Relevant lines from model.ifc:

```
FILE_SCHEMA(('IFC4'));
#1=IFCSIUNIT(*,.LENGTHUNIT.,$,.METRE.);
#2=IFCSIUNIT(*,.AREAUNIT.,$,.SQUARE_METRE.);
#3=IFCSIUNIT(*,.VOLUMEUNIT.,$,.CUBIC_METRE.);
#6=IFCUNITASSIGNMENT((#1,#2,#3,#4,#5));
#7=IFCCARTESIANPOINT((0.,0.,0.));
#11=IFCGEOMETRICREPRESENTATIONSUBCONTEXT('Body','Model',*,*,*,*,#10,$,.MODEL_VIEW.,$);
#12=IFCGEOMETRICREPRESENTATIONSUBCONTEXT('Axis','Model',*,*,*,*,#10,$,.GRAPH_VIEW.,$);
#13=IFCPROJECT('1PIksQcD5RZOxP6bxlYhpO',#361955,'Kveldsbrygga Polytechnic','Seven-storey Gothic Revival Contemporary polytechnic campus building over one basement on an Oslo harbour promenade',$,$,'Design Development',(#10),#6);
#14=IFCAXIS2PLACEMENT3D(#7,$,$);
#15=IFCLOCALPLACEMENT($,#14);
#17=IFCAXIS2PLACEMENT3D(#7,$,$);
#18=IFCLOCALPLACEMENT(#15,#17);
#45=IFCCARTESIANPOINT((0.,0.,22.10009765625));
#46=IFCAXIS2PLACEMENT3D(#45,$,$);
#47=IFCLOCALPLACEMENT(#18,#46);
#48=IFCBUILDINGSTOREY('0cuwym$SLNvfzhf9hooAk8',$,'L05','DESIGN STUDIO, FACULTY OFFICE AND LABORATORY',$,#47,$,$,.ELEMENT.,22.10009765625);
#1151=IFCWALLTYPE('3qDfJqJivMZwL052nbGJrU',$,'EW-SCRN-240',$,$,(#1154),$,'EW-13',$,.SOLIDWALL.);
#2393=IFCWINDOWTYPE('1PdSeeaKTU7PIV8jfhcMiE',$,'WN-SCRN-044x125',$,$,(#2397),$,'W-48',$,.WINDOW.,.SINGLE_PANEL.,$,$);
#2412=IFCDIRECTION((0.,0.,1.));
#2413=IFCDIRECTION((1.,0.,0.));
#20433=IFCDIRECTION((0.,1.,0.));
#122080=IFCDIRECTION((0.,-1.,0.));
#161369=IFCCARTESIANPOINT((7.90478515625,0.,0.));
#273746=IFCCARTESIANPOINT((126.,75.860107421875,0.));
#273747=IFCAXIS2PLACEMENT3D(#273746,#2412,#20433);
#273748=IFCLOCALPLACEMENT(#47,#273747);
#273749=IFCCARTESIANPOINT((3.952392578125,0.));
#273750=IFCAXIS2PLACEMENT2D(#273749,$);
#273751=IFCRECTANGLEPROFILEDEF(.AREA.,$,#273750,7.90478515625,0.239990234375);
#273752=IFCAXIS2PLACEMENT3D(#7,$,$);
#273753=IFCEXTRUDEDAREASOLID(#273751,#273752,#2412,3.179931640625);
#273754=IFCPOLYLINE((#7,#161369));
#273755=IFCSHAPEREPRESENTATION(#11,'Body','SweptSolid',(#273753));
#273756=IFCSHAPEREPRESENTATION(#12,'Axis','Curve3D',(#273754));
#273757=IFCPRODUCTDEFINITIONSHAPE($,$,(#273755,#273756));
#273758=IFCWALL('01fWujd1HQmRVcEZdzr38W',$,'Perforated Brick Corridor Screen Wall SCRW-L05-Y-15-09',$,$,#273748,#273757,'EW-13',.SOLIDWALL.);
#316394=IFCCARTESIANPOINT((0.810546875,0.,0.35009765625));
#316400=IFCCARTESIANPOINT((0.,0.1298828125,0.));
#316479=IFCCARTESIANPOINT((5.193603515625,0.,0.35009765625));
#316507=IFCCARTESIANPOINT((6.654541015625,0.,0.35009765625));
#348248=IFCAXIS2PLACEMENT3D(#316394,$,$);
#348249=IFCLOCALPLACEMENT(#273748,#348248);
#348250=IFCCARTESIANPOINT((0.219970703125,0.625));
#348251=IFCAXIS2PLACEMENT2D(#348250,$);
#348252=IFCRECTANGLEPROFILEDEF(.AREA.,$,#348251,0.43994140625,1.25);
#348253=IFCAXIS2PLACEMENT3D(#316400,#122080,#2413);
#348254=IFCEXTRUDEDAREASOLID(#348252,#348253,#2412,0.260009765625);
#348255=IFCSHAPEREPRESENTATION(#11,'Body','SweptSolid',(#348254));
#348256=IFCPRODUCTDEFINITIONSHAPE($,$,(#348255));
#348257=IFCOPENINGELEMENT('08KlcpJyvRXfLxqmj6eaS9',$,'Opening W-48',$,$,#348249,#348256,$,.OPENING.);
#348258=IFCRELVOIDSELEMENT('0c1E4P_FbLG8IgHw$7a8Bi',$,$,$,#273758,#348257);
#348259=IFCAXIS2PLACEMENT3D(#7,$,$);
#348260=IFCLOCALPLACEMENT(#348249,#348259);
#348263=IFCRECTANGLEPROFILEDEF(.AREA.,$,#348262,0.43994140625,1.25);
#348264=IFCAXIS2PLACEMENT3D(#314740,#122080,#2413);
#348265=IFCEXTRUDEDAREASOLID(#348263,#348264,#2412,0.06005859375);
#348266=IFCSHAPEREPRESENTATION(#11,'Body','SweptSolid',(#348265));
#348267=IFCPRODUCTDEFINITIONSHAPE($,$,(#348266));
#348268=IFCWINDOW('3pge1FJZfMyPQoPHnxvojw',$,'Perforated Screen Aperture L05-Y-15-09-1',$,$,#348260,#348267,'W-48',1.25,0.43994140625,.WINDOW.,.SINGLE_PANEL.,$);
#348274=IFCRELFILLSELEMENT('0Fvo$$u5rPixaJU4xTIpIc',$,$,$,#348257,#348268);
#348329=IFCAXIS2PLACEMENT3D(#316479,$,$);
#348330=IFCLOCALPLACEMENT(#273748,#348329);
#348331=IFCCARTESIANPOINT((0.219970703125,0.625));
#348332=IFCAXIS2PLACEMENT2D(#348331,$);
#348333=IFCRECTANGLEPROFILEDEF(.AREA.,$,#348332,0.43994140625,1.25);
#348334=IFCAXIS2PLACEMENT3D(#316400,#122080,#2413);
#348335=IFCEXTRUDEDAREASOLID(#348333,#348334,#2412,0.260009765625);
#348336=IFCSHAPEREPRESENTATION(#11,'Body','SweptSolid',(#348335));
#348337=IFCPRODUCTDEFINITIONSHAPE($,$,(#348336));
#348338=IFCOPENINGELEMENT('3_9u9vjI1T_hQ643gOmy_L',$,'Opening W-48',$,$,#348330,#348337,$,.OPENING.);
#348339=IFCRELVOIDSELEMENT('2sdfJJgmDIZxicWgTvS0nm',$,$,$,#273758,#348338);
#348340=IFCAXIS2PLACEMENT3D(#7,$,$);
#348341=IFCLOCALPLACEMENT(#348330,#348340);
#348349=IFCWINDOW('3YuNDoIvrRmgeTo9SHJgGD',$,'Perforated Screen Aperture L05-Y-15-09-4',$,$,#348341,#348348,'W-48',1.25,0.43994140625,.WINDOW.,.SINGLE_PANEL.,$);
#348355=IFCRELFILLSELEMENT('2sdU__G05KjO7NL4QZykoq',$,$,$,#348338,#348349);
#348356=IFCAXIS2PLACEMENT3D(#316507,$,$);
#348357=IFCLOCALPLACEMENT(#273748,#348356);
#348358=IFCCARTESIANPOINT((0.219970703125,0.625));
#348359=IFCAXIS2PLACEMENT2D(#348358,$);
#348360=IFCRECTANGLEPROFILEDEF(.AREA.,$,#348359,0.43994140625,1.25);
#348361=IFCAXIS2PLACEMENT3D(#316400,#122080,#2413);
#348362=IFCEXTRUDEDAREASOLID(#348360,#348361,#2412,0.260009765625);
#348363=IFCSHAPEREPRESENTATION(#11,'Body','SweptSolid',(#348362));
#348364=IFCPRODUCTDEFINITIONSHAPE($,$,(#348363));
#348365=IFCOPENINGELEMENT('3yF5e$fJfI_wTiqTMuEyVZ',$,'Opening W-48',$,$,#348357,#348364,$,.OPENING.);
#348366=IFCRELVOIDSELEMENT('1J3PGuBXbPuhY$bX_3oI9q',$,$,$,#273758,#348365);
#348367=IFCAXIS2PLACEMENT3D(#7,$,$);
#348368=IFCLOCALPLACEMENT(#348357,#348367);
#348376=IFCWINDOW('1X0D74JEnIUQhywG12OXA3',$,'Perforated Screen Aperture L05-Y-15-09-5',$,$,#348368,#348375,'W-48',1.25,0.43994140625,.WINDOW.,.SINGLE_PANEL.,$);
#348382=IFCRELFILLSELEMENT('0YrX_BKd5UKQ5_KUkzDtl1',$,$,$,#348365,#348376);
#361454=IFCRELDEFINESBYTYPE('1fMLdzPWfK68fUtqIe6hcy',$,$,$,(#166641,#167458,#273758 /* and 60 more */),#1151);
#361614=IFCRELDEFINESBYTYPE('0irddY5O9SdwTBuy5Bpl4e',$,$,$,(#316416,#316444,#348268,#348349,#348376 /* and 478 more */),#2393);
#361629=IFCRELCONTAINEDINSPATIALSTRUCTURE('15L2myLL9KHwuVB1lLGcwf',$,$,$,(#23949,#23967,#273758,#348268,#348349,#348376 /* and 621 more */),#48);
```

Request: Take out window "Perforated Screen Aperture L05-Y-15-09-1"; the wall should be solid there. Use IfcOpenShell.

```python
import ifcopenshell
import ifcopenshell.api.feature
import ifcopenshell.api.root
import ifcopenshell.geom
import ifcopenshell.util.shape

model = ifcopenshell.open("model.ifc")
settings = ifcopenshell.geom.settings()


def volume(element):
    """Net volume in cubic metres, openings subtracted."""
    shape = ifcopenshell.geom.create_shape(settings, element)
    return ifcopenshell.util.shape.get_volume(shape.geometry)


window = model.by_guid("3pge1FJZfMyPQoPHnxvojw")
opening = window.FillsVoids[0].RelatingOpeningElement
wall = opening.VoidsElements[0].RelatingBuildingElement
before = volume(wall)

ifcopenshell.api.root.remove_product(model, product=window)
ifcopenshell.api.feature.remove_feature(model, feature=opening)

after = volume(wall)

print(f"wall volume {before:.3f} -> {after:.3f} m3")

model.write("model-out.ifc")
```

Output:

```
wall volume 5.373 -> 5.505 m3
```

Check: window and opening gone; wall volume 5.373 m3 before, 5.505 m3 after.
